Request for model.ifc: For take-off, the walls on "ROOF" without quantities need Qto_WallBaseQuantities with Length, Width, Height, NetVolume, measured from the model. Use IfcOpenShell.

First a look at what the model holds.

```python
import ifcopenshell
import ifcopenshell.util.element
import ifcopenshell.util.unit

model = ifcopenshell.open("model.ifc")
print(model.schema)
for unit_type in ("LENGTHUNIT", "AREAUNIT", "VOLUMEUNIT"):
    print(unit_type, ifcopenshell.util.unit.calculate_unit_scale(model, unit_type))
storey = next(s for s in model.by_type("IfcBuildingStorey") if s.Name == "ROOF")
walls = [e for e in ifcopenshell.util.element.get_decomposition(storey) if e.is_a("IfcWall")]
for e in sorted(walls, key=lambda e: e.id()):
    print(e.id(), e.is_a(), e.Name, list(ifcopenshell.util.element.get_psets(e, qtos_only=True)), sep=" | ")
```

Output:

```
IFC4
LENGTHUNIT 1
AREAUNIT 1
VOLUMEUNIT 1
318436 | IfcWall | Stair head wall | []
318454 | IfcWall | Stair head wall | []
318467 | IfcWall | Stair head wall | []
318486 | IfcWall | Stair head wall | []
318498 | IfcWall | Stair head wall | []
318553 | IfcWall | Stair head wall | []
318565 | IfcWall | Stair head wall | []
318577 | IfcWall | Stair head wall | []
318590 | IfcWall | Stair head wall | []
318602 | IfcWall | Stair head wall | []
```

```python
import ifcopenshell
import ifcopenshell.api.pset
import ifcopenshell.geom
import ifcopenshell.util.element
import ifcopenshell.util.shape
import ifcopenshell.util.unit

model = ifcopenshell.open("model.ifc")
unit_scale = ifcopenshell.util.unit.calculate_unit_scale(model)
volume_scale = ifcopenshell.util.unit.calculate_unit_scale(model, "VOLUMEUNIT")
settings = ifcopenshell.geom.settings()

storey = next(s for s in model.by_type("IfcBuildingStorey") if s.Name == "ROOF")
walls = [e for e in ifcopenshell.util.element.get_decomposition(storey) if e.is_a("IfcWall")]

for e in sorted(walls, key=lambda e: e.id()):
    if ifcopenshell.util.element.get_psets(e, qtos_only=True, should_inherit=False):
        continue
    # Geometry comes back in metres, in the element's own axes.
    shape = ifcopenshell.geom.create_shape(settings, e)
    values = {
        "Length": ifcopenshell.util.shape.get_x(shape.geometry) / unit_scale,
        "Width": ifcopenshell.util.shape.get_y(shape.geometry) / unit_scale,
        "Height": ifcopenshell.util.shape.get_z(shape.geometry) / unit_scale,
        "NetVolume": ifcopenshell.util.shape.get_volume(shape.geometry) / volume_scale,
    }
    qto = ifcopenshell.api.pset.add_qto(model, product=e, name="Qto_WallBaseQuantities")
    ifcopenshell.api.pset.edit_qto(model, qto=qto, properties=values)
    print(e.id(), {k: round(v, 3) for k, v in values.items()})

model.write("model_updated.ifc")
```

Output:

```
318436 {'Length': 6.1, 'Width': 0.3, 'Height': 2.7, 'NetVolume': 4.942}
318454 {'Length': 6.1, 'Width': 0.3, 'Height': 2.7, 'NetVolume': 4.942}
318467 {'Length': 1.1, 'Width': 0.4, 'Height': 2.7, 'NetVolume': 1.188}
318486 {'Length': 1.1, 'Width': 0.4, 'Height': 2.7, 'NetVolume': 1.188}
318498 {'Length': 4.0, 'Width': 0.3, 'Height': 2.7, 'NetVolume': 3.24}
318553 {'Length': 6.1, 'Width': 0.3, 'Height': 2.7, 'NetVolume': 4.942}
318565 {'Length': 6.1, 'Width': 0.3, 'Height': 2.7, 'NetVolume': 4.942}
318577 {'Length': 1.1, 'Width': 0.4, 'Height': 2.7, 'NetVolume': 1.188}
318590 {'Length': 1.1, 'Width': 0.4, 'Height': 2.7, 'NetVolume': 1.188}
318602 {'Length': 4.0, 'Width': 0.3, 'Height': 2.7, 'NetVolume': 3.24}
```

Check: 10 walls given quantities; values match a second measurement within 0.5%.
